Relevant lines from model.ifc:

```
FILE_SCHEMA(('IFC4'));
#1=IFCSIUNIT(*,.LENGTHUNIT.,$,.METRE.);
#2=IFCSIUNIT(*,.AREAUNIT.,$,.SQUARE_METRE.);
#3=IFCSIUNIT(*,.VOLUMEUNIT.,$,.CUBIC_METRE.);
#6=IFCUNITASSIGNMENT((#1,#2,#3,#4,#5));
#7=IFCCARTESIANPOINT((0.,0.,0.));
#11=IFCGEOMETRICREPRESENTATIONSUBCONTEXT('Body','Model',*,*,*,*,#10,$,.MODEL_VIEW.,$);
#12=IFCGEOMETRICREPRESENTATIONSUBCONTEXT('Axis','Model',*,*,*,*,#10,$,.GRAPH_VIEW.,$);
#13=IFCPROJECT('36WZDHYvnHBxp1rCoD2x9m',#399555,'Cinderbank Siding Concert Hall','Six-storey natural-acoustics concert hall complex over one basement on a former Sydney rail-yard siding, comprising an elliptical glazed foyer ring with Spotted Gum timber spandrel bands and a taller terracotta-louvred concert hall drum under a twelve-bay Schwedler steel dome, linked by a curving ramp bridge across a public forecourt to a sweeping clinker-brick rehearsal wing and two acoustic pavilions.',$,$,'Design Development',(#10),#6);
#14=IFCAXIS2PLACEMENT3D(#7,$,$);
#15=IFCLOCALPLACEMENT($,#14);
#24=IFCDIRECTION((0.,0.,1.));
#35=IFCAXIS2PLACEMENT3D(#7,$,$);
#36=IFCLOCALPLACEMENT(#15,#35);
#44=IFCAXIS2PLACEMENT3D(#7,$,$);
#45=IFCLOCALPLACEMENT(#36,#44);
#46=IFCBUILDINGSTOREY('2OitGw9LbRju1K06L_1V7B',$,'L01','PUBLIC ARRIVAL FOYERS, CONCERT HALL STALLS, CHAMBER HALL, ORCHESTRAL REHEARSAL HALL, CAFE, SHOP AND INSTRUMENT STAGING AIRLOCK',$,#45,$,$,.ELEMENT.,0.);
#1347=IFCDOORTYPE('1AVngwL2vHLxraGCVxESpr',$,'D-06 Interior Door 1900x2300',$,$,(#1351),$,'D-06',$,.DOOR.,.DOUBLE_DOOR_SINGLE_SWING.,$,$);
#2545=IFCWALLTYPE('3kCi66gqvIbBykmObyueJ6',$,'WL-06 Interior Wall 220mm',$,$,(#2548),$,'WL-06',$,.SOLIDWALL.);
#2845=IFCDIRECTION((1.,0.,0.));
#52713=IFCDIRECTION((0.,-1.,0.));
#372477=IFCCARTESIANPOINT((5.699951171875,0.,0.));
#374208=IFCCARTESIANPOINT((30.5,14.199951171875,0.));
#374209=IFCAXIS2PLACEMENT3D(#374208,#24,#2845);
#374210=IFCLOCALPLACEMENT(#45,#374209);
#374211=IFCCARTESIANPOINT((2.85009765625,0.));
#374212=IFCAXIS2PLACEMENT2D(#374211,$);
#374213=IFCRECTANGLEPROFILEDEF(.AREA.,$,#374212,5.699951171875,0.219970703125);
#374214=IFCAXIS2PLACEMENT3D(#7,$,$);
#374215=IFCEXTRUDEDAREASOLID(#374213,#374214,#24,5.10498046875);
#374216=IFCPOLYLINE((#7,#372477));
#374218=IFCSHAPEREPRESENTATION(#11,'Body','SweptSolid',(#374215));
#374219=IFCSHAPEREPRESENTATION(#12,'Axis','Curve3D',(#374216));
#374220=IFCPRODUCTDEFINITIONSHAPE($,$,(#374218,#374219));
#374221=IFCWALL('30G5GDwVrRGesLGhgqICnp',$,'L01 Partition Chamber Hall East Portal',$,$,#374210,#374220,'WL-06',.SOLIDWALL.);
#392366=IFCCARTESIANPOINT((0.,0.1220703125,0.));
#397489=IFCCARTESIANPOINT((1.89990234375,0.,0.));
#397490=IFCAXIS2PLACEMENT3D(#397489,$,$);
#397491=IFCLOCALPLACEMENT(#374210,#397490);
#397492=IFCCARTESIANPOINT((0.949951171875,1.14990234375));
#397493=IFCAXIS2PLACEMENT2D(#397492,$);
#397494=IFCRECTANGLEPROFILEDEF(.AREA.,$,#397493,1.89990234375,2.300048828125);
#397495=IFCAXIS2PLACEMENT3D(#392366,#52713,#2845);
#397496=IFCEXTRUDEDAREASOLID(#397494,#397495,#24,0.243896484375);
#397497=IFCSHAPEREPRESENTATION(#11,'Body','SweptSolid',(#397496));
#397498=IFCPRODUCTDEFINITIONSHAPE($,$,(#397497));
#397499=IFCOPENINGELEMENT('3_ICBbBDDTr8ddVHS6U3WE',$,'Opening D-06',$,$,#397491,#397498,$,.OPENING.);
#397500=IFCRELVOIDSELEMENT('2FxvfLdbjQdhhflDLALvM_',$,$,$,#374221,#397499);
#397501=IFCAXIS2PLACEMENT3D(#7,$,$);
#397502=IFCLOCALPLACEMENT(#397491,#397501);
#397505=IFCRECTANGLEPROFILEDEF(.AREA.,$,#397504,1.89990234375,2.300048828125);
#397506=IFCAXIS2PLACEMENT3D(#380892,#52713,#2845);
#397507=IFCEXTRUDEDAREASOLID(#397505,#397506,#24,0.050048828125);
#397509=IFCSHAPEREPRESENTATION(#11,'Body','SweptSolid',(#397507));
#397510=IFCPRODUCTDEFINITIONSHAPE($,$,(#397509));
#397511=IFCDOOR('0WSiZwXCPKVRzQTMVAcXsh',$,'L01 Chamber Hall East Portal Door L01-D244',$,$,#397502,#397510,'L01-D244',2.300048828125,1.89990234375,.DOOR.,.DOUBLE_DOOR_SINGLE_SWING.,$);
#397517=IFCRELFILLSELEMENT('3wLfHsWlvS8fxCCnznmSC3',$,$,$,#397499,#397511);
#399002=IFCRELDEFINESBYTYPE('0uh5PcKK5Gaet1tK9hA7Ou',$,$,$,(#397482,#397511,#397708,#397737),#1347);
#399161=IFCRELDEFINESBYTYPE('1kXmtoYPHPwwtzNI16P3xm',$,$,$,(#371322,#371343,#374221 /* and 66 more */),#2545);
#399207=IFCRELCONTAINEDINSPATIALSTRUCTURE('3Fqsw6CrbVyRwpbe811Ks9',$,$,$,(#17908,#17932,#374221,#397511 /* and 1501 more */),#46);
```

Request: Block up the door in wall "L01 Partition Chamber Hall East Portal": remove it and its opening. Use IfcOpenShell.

```python
import ifcopenshell
import ifcopenshell.api.feature
import ifcopenshell.api.root
import ifcopenshell.geom
import ifcopenshell.util.shape

model = ifcopenshell.open("model.ifc")
settings = ifcopenshell.geom.settings()


def volume(element):
    """Net volume in cubic metres, openings subtracted."""
    shape = ifcopenshell.geom.create_shape(settings, element)
    return ifcopenshell.util.shape.get_volume(shape.geometry)


door = model.by_id(397511)
opening = door.FillsVoids[0].RelatingOpeningElement
wall = opening.VoidsElements[0].RelatingBuildingElement
before = volume(wall)

ifcopenshell.api.root.remove_product(model, product=door)
ifcopenshell.api.feature.remove_feature(model, feature=opening)

after = volume(wall)

print(f"wall volume {before:.3f} -> {after:.3f} m3")

model.write("model_rev.ifc")
```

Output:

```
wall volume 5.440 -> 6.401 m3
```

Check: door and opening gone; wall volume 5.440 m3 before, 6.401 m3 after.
